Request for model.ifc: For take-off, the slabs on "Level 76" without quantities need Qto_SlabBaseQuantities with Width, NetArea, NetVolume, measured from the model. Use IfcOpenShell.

First a look at what the model holds.

```python
import ifcopenshell
import ifcopenshell.util.element
import ifcopenshell.util.unit

model = ifcopenshell.open("model.ifc")
print(model.schema)
for unit_type in ("LENGTHUNIT", "AREAUNIT", "VOLUMEUNIT"):
    print(unit_type, ifcopenshell.util.unit.calculate_unit_scale(model, unit_type))
storey = next(s for s in model.by_type("IfcBuildingStorey") if s.Name == "Level 76")
slabs = [e for e in ifcopenshell.util.element.get_decomposition(storey) if e.is_a("IfcSlab")]
for e in sorted(slabs, key=lambda e: e.id()):
    print(e.id(), e.is_a(), e.Name, list(ifcopenshell.util.element.get_psets(e, qtos_only=True)), sep=" | ")
```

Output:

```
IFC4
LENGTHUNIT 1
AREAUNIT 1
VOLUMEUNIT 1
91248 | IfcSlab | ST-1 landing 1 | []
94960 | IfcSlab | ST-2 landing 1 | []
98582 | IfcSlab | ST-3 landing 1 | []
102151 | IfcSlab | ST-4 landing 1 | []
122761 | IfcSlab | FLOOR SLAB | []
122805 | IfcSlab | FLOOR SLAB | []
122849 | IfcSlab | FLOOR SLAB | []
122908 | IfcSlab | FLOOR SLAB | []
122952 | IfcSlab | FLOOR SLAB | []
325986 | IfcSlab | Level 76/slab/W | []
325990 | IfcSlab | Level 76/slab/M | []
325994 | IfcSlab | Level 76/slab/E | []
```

```python
import ifcopenshell
import ifcopenshell.api.pset
import ifcopenshell.geom
import ifcopenshell.util.element
import ifcopenshell.util.shape
import ifcopenshell.util.unit

model = ifcopenshell.open("model.ifc")
unit_scale = ifcopenshell.util.unit.calculate_unit_scale(model)
area_scale = ifcopenshell.util.unit.calculate_unit_scale(model, "AREAUNIT")
volume_scale = ifcopenshell.util.unit.calculate_unit_scale(model, "VOLUMEUNIT")
settings = ifcopenshell.geom.settings()

storey = next(s for s in model.by_type("IfcBuildingStorey") if s.Name == "Level 76")
slabs = [e for e in ifcopenshell.util.element.get_decomposition(storey) if e.is_a("IfcSlab")]

for e in sorted(slabs, key=lambda e: e.id()):
    if ifcopenshell.util.element.get_psets(e, qtos_only=True, should_inherit=False):
        continue
    # Geometry comes back in metres, in the element's own axes.
    shape = ifcopenshell.geom.create_shape(settings, e)
    values = {
        "Width": ifcopenshell.util.shape.get_z(shape.geometry) / unit_scale,
        "NetArea": ifcopenshell.util.shape.get_footprint_area(shape.geometry) / area_scale,
        "NetVolume": ifcopenshell.util.shape.get_volume(shape.geometry) / volume_scale,
    }
    qto = ifcopenshell.api.pset.add_qto(model, product=e, name="Qto_SlabBaseQuantities")
    ifcopenshell.api.pset.edit_qto(model, qto=qto, properties=values)
    print(e.id(), {k: round(v, 3) for k, v in values.items()})

model.write("model_updated.ifc")
```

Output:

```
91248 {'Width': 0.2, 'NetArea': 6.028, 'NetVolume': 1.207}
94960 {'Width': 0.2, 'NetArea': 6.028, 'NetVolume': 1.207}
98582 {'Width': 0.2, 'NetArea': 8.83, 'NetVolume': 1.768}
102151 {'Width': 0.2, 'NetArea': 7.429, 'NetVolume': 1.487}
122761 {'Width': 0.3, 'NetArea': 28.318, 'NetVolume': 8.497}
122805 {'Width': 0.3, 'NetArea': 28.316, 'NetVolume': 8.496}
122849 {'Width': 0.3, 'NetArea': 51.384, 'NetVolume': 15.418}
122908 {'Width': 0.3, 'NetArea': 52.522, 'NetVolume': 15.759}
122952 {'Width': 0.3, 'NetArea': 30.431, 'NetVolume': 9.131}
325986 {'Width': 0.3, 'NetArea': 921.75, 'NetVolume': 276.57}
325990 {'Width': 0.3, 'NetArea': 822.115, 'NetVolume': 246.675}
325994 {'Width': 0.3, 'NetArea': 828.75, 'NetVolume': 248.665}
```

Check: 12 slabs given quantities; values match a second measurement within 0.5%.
